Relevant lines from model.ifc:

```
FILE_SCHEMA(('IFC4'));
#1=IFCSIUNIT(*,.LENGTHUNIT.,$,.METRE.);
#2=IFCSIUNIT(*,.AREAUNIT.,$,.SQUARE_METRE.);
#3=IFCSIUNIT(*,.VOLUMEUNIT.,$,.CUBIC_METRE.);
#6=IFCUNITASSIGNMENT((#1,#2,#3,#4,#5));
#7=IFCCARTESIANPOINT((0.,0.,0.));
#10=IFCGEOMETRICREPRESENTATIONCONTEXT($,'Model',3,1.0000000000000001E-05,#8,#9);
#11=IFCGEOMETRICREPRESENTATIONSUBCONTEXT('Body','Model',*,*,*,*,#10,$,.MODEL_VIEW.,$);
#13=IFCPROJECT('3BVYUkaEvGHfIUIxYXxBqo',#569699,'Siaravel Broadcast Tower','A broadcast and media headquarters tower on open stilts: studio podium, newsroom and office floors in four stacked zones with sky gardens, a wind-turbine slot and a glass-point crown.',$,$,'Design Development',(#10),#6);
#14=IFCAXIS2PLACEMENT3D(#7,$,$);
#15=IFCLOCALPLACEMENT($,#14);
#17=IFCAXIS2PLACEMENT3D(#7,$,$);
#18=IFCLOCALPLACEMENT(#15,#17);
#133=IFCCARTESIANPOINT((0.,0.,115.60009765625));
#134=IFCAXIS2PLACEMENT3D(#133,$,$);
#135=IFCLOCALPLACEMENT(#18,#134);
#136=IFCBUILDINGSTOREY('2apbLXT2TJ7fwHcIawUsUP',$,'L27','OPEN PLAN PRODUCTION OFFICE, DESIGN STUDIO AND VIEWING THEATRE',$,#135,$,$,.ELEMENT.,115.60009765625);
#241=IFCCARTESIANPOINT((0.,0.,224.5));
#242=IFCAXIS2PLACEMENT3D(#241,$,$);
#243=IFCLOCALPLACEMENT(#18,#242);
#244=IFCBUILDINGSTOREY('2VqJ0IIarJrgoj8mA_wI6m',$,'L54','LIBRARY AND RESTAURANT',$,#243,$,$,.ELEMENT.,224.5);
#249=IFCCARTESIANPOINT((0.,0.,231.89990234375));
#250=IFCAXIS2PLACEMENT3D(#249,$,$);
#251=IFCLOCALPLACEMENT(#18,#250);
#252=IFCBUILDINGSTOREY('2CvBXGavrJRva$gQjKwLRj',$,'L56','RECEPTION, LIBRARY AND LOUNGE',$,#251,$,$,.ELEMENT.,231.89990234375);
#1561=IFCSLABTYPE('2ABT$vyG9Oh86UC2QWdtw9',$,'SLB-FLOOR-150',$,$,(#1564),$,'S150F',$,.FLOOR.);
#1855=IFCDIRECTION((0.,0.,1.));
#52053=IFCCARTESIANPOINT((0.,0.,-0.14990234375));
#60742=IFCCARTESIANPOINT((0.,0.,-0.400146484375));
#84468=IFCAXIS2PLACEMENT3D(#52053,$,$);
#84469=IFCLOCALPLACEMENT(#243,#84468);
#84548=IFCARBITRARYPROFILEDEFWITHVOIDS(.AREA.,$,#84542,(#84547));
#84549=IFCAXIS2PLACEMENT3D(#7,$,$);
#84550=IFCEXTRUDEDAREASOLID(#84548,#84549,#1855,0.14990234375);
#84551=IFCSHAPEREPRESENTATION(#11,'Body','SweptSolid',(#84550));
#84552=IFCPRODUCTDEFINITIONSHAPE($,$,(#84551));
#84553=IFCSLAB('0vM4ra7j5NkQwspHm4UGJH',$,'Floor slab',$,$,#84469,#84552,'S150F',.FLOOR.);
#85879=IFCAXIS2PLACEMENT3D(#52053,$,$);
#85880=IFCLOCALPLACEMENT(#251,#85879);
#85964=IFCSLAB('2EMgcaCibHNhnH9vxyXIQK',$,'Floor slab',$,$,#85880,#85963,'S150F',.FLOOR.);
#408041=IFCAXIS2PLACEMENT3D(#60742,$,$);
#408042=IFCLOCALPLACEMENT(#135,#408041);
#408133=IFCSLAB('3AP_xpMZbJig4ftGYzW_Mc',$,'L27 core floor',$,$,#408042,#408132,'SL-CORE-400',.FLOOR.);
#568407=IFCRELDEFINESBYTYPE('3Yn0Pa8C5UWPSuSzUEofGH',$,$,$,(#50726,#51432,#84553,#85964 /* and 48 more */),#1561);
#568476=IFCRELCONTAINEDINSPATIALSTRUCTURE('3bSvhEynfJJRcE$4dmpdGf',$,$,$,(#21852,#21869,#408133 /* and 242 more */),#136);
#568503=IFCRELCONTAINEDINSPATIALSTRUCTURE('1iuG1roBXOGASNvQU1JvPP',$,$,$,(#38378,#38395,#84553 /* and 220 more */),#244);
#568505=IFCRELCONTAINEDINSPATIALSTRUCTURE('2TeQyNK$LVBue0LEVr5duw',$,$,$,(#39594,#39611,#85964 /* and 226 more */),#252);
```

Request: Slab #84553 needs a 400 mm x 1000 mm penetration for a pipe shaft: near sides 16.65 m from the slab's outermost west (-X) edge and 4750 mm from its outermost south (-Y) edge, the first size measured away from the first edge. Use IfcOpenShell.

```python
import numpy as np
import ifcopenshell
import ifcopenshell.api.feature
import ifcopenshell.api.geometry
import ifcopenshell.api.root
import ifcopenshell.geom
import ifcopenshell.util.placement
import ifcopenshell.util.representation
import ifcopenshell.util.shape
import ifcopenshell.util.unit

model = ifcopenshell.open("model.ifc")
unit_scale = ifcopenshell.util.unit.calculate_unit_scale(model)
settings = ifcopenshell.geom.settings()


def volume(element):
    """Net volume in cubic metres, openings subtracted."""
    shape = ifcopenshell.geom.create_shape(settings, element)
    return ifcopenshell.util.shape.get_volume(shape.geometry)


slab = model.by_id(84553)
before = volume(slab)

# Extent in the slab's own axes, in metres. The edges named are its -X and -Y sides.
slab_shape = ifcopenshell.geom.create_shape(settings, slab)
vertices = ifcopenshell.util.shape.get_vertices(slab_shape.geometry)
x_min, y_min, bottom = vertices.min(axis=0)
top = vertices[:, 2].max()

opening = ifcopenshell.api.root.create_entity(model, ifc_class="IfcOpeningElement", name="Pipe shaft opening", predefined_type="OPENING")
context = ifcopenshell.util.representation.get_context(model, "Model", "Body", "MODEL_VIEW")
width, depth = 0.4, 1
outline = [(0.0, 0.0), (width, 0.0), (width, depth), (0.0, depth), (0.0, 0.0)]
# Overshoot both faces by 50 mm so the cut is clean.
shape = ifcopenshell.api.geometry.add_slab_representation(
    model, context=context, depth=top - bottom + 0.1, polyline=outline
)
ifcopenshell.api.geometry.assign_representation(model, product=opening, representation=shape)

matrix = ifcopenshell.util.placement.get_local_placement(slab.ObjectPlacement)
matrix[:, 3] = matrix @ np.append(np.array([x_min + 16.65, y_min + 4.75, bottom - 0.05]) / unit_scale, 1.0)
ifcopenshell.api.geometry.edit_object_placement(model, product=opening, matrix=matrix, is_si=False)
ifcopenshell.api.feature.add_feature(model, feature=opening, element=slab)

after = volume(slab)

print(f"slab volume {before:.3f} -> {after:.3f} m3")

model.write("model_edited.ifc")
```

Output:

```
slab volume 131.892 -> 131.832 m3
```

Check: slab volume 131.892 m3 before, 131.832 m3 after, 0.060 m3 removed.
